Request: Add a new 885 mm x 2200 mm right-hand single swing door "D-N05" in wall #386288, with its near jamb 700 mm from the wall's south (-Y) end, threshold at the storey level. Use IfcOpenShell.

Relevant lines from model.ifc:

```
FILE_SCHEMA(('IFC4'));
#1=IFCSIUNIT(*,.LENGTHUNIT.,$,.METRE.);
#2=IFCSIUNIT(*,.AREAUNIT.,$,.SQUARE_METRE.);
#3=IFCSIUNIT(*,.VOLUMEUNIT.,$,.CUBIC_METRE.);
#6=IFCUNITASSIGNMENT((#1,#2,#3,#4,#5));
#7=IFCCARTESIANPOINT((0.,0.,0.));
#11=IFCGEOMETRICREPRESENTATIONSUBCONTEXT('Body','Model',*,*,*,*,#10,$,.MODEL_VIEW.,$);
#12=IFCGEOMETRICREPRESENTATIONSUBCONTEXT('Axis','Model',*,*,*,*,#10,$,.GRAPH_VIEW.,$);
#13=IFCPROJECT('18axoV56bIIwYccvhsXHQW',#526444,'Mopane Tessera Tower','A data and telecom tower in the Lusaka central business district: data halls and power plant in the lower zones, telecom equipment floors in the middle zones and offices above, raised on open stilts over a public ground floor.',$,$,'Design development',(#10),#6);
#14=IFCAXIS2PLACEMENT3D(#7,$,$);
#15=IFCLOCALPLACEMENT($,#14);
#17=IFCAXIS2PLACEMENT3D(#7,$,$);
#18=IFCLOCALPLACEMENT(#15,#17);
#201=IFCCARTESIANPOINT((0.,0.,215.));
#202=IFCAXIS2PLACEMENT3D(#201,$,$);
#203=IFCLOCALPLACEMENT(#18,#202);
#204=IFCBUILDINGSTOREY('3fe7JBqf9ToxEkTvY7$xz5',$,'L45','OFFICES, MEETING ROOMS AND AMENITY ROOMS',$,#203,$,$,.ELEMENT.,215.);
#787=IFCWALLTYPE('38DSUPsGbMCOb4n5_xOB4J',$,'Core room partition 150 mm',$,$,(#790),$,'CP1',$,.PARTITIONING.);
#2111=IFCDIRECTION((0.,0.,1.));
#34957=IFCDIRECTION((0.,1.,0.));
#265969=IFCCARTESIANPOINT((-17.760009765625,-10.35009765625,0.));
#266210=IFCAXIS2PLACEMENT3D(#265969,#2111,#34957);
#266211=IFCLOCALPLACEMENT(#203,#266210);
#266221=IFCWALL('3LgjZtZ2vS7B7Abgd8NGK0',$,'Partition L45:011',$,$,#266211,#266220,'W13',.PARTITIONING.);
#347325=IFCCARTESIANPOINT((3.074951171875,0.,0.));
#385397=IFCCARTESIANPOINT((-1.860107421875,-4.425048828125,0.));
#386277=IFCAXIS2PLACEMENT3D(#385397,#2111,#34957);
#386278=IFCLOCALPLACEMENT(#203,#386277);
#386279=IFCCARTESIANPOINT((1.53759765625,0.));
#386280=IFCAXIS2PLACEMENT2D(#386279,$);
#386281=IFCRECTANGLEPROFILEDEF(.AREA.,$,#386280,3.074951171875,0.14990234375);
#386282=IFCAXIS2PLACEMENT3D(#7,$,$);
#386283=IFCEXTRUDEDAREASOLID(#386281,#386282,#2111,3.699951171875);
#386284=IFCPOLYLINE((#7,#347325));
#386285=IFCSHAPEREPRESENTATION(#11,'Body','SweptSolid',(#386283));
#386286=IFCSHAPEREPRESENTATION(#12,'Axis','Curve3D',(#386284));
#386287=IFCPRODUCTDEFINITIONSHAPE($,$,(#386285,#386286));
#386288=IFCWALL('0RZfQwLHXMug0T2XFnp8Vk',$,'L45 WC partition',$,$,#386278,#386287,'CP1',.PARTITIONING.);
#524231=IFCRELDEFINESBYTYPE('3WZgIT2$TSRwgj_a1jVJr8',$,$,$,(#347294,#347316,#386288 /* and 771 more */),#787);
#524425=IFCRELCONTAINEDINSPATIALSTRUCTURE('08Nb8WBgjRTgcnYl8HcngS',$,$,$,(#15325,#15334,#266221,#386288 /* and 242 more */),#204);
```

```python
import numpy as np
import ifcopenshell
import ifcopenshell.api.feature
import ifcopenshell.api.geometry
import ifcopenshell.api.root
import ifcopenshell.api.spatial
import ifcopenshell.geom
import ifcopenshell.util.element
import ifcopenshell.util.placement
import ifcopenshell.util.representation
import ifcopenshell.util.shape
import ifcopenshell.util.unit

model = ifcopenshell.open("model.ifc")
unit_scale = ifcopenshell.util.unit.calculate_unit_scale(model)
settings = ifcopenshell.geom.settings()


def volume(element):
    """Net volume in cubic metres, openings subtracted."""
    shape = ifcopenshell.geom.create_shape(settings, element)
    return ifcopenshell.util.shape.get_volume(shape.geometry)


wall = model.by_id(386288)
storey = ifcopenshell.util.element.get_container(wall, ifc_class="IfcBuildingStorey")
context = ifcopenshell.util.representation.get_context(model, "Model", "Body", "MODEL_VIEW")
before = volume(wall)

width, height, from_end, sill = 0.885, 2.2, 0.7, 0.0  # metres

# The wall runs along its own X axis, and the end named is its -X end.
wall_shape = ifcopenshell.geom.create_shape(settings, wall)
x, y, z = ifcopenshell.util.shape.get_vertices(wall_shape.geometry).T
start = x.min() + from_end
face, thickness = float(y.min()), float(y.max() - y.min())
wall_matrix = ifcopenshell.util.placement.get_local_placement(wall.ObjectPlacement)
level = ifcopenshell.util.placement.get_local_placement(storey.ObjectPlacement)[2, 3]


def in_wall(x, y):
    """Placement at x, y metres in the wall's axes, at sill height."""
    matrix = wall_matrix.copy()
    matrix[:, 3] = wall_matrix @ np.array([x / unit_scale, y / unit_scale, 0.0, 1.0])
    matrix[2, 3] = level + sill / unit_scale
    return matrix


# Opening: a box that overshoots both wall faces by 50 mm.
opening = ifcopenshell.api.root.create_entity(model, ifc_class="IfcOpeningElement", predefined_type="OPENING")
box = ifcopenshell.api.geometry.add_wall_representation(
    model, context=context, length=width, height=height, thickness=thickness + 0.1
)
ifcopenshell.api.geometry.assign_representation(model, product=opening, representation=box)
ifcopenshell.api.geometry.edit_object_placement(model, product=opening, matrix=in_wall(start, face - 0.05), is_si=False)
ifcopenshell.api.feature.add_feature(model, feature=opening, element=wall)

door = ifcopenshell.api.root.create_entity(model, ifc_class="IfcDoor", name="D-N05", predefined_type="DOOR")
door.OverallWidth, door.OverallHeight = width / unit_scale, height / unit_scale
door.OperationType = "SINGLE_SWING_RIGHT"
body = ifcopenshell.api.geometry.add_door_representation(
    model,
    context=context,
    overall_width=door.OverallWidth,
    overall_height=door.OverallHeight,
    operation_type="SINGLE_SWING_RIGHT",
    lining_properties={"LiningDepth": thickness / unit_scale, "ThresholdDepth": thickness / unit_scale},
)
ifcopenshell.api.geometry.assign_representation(model, product=door, representation=body)
ifcopenshell.api.spatial.assign_container(model, products=[door], relating_structure=storey)
ifcopenshell.api.feature.add_filling(model, opening=opening, element=door)

# The lining spans the wall, so the door starts at the wall face.
ifcopenshell.api.geometry.edit_object_placement(model, product=door, matrix=in_wall(start, face), is_si=False)

after = volume(wall)

print(f"wall volume {before:.3f} -> {after:.3f} m3")

model.write("model_edited.ifc")
```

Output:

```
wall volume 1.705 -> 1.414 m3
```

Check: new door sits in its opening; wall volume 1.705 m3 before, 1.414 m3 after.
